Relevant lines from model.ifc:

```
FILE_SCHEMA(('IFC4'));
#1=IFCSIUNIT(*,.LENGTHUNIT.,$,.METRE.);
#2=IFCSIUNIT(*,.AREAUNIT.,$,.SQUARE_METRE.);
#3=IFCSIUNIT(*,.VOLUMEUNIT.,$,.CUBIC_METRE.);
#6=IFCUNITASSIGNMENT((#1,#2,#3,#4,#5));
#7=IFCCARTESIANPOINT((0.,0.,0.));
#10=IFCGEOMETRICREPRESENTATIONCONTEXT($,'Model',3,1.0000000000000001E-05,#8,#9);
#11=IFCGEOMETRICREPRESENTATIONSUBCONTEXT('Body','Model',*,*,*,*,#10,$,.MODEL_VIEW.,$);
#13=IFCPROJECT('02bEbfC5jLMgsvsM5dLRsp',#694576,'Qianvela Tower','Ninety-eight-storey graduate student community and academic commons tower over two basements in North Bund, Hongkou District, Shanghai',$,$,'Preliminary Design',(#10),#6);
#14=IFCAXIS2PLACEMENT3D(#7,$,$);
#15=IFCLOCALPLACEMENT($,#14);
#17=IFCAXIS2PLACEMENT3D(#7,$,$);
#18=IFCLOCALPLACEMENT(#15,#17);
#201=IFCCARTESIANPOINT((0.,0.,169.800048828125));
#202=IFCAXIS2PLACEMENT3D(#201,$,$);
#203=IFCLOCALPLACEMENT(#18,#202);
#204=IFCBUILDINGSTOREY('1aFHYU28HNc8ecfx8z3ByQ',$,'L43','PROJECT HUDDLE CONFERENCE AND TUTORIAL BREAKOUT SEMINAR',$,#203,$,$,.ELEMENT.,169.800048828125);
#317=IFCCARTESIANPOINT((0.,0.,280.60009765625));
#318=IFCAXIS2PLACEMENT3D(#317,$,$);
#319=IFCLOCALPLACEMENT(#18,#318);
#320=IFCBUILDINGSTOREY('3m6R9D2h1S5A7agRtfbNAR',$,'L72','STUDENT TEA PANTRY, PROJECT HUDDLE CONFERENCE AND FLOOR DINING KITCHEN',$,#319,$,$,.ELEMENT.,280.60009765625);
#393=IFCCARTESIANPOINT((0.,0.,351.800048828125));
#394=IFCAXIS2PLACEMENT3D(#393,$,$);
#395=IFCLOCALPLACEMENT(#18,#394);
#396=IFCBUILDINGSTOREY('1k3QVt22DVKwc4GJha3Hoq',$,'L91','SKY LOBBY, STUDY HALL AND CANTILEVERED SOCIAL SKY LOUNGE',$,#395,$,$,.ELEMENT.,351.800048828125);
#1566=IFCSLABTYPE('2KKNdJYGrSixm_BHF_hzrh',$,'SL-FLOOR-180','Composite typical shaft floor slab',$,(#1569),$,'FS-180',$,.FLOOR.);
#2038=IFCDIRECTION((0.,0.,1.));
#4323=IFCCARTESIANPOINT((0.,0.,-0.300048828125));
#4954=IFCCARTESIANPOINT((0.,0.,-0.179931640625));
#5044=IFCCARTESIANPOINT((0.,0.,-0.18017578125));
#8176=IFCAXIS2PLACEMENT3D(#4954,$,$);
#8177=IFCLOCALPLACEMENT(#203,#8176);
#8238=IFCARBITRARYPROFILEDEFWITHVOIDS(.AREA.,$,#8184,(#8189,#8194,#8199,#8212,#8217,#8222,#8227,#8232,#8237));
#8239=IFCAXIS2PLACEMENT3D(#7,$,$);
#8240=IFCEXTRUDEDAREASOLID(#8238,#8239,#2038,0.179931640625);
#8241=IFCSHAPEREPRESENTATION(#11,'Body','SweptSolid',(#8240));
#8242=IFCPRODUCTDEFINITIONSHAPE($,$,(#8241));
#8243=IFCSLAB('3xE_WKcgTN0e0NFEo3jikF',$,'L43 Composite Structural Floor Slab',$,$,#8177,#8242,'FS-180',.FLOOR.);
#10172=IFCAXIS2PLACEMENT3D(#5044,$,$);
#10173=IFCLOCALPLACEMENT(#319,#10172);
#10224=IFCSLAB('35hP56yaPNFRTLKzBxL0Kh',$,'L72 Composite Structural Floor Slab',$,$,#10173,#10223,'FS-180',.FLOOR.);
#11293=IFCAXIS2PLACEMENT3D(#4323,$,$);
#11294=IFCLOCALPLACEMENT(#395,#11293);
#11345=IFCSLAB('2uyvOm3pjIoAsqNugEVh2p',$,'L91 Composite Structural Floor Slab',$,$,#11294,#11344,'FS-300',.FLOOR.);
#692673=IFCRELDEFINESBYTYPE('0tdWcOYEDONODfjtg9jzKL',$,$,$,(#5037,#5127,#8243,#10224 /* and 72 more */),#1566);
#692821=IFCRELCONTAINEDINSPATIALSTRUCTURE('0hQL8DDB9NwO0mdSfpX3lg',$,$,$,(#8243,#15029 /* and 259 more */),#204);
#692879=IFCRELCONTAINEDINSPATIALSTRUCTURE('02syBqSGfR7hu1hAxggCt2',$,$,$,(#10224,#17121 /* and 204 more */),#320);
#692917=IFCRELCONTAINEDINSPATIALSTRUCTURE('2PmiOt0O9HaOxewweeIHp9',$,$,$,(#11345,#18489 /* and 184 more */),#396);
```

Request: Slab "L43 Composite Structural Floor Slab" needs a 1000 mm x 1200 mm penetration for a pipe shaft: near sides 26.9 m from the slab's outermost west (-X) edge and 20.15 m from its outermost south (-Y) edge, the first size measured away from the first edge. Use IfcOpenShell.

```python
import numpy as np
import ifcopenshell
import ifcopenshell.api.feature
import ifcopenshell.api.geometry
import ifcopenshell.api.root
import ifcopenshell.geom
import ifcopenshell.util.placement
import ifcopenshell.util.representation
import ifcopenshell.util.shape
import ifcopenshell.util.unit

model = ifcopenshell.open("model.ifc")
unit_scale = ifcopenshell.util.unit.calculate_unit_scale(model)
settings = ifcopenshell.geom.settings()


def volume(element):
    """Net volume in cubic metres, openings subtracted."""
    shape = ifcopenshell.geom.create_shape(settings, element)
    return ifcopenshell.util.shape.get_volume(shape.geometry)


slab = model.by_id(8243)
before = volume(slab)

# Extent in the slab's own axes, in metres. The edges named are its -X and -Y sides.
slab_shape = ifcopenshell.geom.create_shape(settings, slab)
vertices = ifcopenshell.util.shape.get_vertices(slab_shape.geometry)
x_min, y_min, bottom = vertices.min(axis=0)
top = vertices[:, 2].max()

opening = ifcopenshell.api.root.create_entity(model, ifc_class="IfcOpeningElement", name="Pipe shaft opening", predefined_type="OPENING")
context = ifcopenshell.util.representation.get_context(model, "Model", "Body", "MODEL_VIEW")
width, depth = 1, 1.2
outline = [(0.0, 0.0), (width, 0.0), (width, depth), (0.0, depth), (0.0, 0.0)]
# Overshoot both faces by 50 mm so the cut is clean.
shape = ifcopenshell.api.geometry.add_slab_representation(
    model, context=context, depth=top - bottom + 0.1, polyline=outline
)
ifcopenshell.api.geometry.assign_representation(model, product=opening, representation=shape)

matrix = ifcopenshell.util.placement.get_local_placement(slab.ObjectPlacement)
matrix[:, 3] = matrix @ np.append(np.array([x_min + 26.9, y_min + 20.15, bottom - 0.05]) / unit_scale, 1.0)
ifcopenshell.api.geometry.edit_object_placement(model, product=opening, matrix=matrix, is_si=False)
ifcopenshell.api.feature.add_feature(model, feature=opening, element=slab)

after = volume(slab)

print(f"slab volume {before:.3f} -> {after:.3f} m3")

model.write("model_updated.ifc")
```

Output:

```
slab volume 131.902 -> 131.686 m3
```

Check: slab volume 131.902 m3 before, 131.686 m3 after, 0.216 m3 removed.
